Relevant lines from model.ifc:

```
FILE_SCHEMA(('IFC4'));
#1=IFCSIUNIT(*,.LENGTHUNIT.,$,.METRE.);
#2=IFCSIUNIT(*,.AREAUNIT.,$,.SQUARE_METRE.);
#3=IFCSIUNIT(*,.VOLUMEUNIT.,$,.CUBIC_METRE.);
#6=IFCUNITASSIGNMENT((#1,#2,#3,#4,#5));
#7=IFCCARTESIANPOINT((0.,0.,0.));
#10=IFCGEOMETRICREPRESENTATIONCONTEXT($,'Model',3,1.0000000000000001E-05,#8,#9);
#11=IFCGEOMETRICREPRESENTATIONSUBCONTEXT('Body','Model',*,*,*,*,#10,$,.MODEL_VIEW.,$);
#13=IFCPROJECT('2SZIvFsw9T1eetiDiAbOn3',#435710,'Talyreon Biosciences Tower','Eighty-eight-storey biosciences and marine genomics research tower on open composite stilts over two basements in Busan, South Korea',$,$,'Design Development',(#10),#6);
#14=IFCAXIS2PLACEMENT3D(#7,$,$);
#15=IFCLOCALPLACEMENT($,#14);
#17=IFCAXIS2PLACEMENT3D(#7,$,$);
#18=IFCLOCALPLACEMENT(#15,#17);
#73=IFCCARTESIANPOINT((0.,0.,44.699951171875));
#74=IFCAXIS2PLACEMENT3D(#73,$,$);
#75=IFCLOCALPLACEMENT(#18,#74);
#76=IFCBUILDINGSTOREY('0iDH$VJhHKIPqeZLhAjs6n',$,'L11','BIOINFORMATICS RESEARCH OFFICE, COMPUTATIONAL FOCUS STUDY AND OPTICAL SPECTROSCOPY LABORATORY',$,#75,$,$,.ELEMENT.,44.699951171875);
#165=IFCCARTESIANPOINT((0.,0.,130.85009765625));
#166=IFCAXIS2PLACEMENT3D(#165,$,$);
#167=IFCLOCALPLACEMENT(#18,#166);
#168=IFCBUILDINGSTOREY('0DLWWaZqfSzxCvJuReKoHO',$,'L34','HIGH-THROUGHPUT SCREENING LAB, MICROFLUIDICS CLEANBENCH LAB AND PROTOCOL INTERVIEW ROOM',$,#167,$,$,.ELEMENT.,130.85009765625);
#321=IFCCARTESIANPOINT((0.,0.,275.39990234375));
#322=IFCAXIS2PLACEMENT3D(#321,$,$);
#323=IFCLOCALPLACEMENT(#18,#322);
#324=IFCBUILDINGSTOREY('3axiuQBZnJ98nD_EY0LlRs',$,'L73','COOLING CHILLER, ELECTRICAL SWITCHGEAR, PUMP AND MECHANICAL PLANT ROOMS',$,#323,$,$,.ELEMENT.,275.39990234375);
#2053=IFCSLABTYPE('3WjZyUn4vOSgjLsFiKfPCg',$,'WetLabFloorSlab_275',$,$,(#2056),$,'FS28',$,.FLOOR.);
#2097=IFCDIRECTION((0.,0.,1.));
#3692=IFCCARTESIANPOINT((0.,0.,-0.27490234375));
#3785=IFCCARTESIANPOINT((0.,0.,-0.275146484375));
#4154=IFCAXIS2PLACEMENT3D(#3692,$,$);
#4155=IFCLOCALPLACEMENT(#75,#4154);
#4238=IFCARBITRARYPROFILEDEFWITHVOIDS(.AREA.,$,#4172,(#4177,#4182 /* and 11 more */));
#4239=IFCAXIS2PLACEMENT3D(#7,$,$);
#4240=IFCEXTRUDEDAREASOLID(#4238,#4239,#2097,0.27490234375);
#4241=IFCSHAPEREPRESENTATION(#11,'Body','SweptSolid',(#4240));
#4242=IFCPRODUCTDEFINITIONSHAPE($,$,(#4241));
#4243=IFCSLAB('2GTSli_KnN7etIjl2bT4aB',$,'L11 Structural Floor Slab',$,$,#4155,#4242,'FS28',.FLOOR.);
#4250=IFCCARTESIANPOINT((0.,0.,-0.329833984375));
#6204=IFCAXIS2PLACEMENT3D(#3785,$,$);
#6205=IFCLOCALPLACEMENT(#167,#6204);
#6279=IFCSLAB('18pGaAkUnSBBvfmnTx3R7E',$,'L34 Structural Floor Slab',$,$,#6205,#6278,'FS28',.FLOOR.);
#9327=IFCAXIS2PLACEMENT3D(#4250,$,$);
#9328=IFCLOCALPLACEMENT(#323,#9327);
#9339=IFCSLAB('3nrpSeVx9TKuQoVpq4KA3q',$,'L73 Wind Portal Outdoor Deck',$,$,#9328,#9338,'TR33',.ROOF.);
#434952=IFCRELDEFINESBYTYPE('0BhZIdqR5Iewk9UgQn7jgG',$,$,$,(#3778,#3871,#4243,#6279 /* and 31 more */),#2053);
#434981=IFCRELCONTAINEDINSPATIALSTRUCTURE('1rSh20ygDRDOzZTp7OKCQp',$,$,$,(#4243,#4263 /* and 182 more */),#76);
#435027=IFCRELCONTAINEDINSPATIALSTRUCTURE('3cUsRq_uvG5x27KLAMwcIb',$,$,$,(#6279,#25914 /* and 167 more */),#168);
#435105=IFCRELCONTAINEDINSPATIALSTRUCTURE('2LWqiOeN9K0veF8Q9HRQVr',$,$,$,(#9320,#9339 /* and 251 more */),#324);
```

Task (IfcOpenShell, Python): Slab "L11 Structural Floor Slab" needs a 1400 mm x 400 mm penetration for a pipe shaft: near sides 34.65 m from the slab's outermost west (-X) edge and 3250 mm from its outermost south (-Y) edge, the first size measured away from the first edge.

```python
import numpy as np
import ifcopenshell
import ifcopenshell.api.feature
import ifcopenshell.api.geometry
import ifcopenshell.api.root
import ifcopenshell.geom
import ifcopenshell.util.placement
import ifcopenshell.util.representation
import ifcopenshell.util.shape
import ifcopenshell.util.unit

model = ifcopenshell.open("model.ifc")
unit_scale = ifcopenshell.util.unit.calculate_unit_scale(model)
settings = ifcopenshell.geom.settings()


def volume(element):
    """Net volume in cubic metres, openings subtracted."""
    shape = ifcopenshell.geom.create_shape(settings, element)
    return ifcopenshell.util.shape.get_volume(shape.geometry)


slab = model.by_guid("2GTSli_KnN7etIjl2bT4aB")
before = volume(slab)

# Extent in the slab's own axes, in metres. The edges named are its -X and -Y sides.
slab_shape = ifcopenshell.geom.create_shape(settings, slab)
vertices = ifcopenshell.util.shape.get_vertices(slab_shape.geometry)
x_min, y_min, bottom = vertices.min(axis=0)
top = vertices[:, 2].max()

opening = ifcopenshell.api.root.create_entity(model, ifc_class="IfcOpeningElement", name="Pipe shaft opening", predefined_type="OPENING")
context = ifcopenshell.util.representation.get_context(model, "Model", "Body", "MODEL_VIEW")
width, depth = 1.4, 0.4
outline = [(0.0, 0.0), (width, 0.0), (width, depth), (0.0, depth), (0.0, 0.0)]
# Overshoot both faces by 50 mm so the cut is clean.
shape = ifcopenshell.api.geometry.add_slab_representation(
    model, context=context, depth=top - bottom + 0.1, polyline=outline
)
ifcopenshell.api.geometry.assign_representation(model, product=opening, representation=shape)

matrix = ifcopenshell.util.placement.get_local_placement(slab.ObjectPlacement)
matrix[:, 3] = matrix @ np.append(np.array([x_min + 34.65, y_min + 3.25, bottom - 0.05]) / unit_scale, 1.0)
ifcopenshell.api.geometry.edit_object_placement(model, product=opening, matrix=matrix, is_si=False)
ifcopenshell.api.feature.add_feature(model, feature=opening, element=slab)

after = volume(slab)

print(f"slab volume {before:.3f} -> {after:.3f} m3")

model.write("model_v2.ifc")
```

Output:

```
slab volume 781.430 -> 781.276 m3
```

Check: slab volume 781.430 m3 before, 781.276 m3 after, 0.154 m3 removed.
